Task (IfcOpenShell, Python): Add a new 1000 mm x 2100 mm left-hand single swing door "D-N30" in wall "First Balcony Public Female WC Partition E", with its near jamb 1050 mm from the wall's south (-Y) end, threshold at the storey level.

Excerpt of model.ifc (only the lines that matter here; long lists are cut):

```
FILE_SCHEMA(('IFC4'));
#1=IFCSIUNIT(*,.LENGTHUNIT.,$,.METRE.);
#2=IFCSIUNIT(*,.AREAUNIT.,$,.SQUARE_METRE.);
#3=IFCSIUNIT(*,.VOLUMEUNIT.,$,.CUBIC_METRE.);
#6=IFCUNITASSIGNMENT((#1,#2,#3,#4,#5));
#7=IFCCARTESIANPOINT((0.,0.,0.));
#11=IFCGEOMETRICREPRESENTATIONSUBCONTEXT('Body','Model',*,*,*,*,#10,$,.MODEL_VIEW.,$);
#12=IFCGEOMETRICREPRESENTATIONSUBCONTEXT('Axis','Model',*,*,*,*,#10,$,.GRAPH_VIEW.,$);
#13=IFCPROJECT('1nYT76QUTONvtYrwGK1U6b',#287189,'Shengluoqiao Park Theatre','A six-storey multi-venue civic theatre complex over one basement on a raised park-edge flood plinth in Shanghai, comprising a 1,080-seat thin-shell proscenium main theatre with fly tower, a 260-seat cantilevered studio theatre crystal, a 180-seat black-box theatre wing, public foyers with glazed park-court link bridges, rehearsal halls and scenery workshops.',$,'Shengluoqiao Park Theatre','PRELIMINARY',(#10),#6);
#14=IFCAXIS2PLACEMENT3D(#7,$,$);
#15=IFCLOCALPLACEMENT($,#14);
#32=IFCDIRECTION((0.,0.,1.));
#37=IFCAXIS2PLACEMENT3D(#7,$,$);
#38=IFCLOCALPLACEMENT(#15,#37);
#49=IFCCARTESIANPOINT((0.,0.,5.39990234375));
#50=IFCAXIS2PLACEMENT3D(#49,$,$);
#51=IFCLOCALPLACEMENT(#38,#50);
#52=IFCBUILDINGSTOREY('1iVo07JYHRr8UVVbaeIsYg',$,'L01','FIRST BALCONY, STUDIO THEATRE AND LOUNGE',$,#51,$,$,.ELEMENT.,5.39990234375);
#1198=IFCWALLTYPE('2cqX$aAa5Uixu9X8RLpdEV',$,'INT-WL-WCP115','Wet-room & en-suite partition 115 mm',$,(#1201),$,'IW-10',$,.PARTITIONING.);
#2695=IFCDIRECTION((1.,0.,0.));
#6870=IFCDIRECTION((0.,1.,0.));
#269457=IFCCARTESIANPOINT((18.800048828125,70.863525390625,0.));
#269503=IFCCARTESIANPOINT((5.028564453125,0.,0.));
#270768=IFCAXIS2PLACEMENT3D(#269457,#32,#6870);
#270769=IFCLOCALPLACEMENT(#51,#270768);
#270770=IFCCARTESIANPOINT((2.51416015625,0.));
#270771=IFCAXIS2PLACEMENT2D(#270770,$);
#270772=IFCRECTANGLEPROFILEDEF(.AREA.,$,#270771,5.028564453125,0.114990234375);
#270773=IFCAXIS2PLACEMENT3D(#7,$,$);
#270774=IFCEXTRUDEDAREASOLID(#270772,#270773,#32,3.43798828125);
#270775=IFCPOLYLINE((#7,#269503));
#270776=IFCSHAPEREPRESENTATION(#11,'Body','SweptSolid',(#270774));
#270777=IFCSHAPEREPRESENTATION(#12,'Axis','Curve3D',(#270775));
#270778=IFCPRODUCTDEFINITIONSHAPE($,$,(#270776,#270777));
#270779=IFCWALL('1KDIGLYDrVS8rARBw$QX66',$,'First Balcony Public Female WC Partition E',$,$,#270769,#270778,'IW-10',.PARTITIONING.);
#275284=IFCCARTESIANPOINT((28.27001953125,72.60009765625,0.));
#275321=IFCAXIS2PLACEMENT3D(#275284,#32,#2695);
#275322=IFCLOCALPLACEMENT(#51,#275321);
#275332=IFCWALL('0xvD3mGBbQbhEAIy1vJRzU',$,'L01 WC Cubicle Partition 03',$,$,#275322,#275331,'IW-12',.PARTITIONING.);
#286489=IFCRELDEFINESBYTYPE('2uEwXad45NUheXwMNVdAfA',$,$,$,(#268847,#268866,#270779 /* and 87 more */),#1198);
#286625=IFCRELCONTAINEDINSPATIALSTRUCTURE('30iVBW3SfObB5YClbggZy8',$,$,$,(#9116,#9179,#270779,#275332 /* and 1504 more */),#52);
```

```python
import numpy as np
import ifcopenshell
import ifcopenshell.api.feature
import ifcopenshell.api.geometry
import ifcopenshell.api.root
import ifcopenshell.api.spatial
import ifcopenshell.geom
import ifcopenshell.util.element
import ifcopenshell.util.placement
import ifcopenshell.util.representation
import ifcopenshell.util.shape
import ifcopenshell.util.unit

model = ifcopenshell.open("model.ifc")
unit_scale = ifcopenshell.util.unit.calculate_unit_scale(model)
settings = ifcopenshell.geom.settings()


def volume(element):
    """Net volume in cubic metres, openings subtracted."""
    shape = ifcopenshell.geom.create_shape(settings, element)
    return ifcopenshell.util.shape.get_volume(shape.geometry)


wall = model.by_guid("1KDIGLYDrVS8rARBw$QX66")
storey = ifcopenshell.util.element.get_container(wall, ifc_class="IfcBuildingStorey")
context = ifcopenshell.util.representation.get_context(model, "Model", "Body", "MODEL_VIEW")
before = volume(wall)

width, height, from_end, sill = 1, 2.1, 1.05, 0.0  # metres

# The wall runs along its own X axis, and the end named is its -X end.
wall_shape = ifcopenshell.geom.create_shape(settings, wall)
x, y, z = ifcopenshell.util.shape.get_vertices(wall_shape.geometry).T
start = x.min() + from_end
face, thickness = float(y.min()), float(y.max() - y.min())
wall_matrix = ifcopenshell.util.placement.get_local_placement(wall.ObjectPlacement)
level = ifcopenshell.util.placement.get_local_placement(storey.ObjectPlacement)[2, 3]


def in_wall(x, y):
    """Placement at x, y metres in the wall's axes, at sill height."""
    matrix = wall_matrix.copy()
    matrix[:, 3] = wall_matrix @ np.array([x / unit_scale, y / unit_scale, 0.0, 1.0])
    matrix[2, 3] = level + sill / unit_scale
    return matrix


# Opening: a box that overshoots both wall faces by 50 mm.
opening = ifcopenshell.api.root.create_entity(model, ifc_class="IfcOpeningElement", predefined_type="OPENING")
box = ifcopenshell.api.geometry.add_wall_representation(
    model, context=context, length=width, height=height, thickness=thickness + 0.1
)
ifcopenshell.api.geometry.assign_representation(model, product=opening, representation=box)
ifcopenshell.api.geometry.edit_object_placement(model, product=opening, matrix=in_wall(start, face - 0.05), is_si=False)
ifcopenshell.api.feature.add_feature(model, feature=opening, element=wall)

door = ifcopenshell.api.root.create_entity(model, ifc_class="IfcDoor", name="D-N30", predefined_type="DOOR")
door.OverallWidth, door.OverallHeight = width / unit_scale, height / unit_scale
door.OperationType = "SINGLE_SWING_LEFT"
body = ifcopenshell.api.geometry.add_door_representation(
    model,
    context=context,
    overall_width=door.OverallWidth,
    overall_height=door.OverallHeight,
    operation_type="SINGLE_SWING_LEFT",
    lining_properties={"LiningDepth": thickness / unit_scale, "ThresholdDepth": thickness / unit_scale},
)
ifcopenshell.api.geometry.assign_representation(model, product=door, representation=body)
ifcopenshell.api.spatial.assign_container(model, products=[door], relating_structure=storey)
ifcopenshell.api.feature.add_filling(model, opening=opening, element=door)

# The lining spans the wall, so the door starts at the wall face.
ifcopenshell.api.geometry.edit_object_placement(model, product=door, matrix=in_wall(start, face), is_si=False)

after = volume(wall)

print(f"wall volume {before:.3f} -> {after:.3f} m3")

model.write("model_rev.ifc")
```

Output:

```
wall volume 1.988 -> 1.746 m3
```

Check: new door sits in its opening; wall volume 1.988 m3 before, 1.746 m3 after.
